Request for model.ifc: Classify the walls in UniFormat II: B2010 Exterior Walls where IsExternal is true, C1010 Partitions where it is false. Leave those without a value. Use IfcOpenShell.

First a look at what the model holds.

```python
import ifcopenshell
import ifcopenshell.util.element

model = ifcopenshell.open("model.ifc")
print(model.schema)
print("classifications:", [c.Name for c in model.by_type("IfcClassification")])
values = [ifcopenshell.util.element.get_pset(e, "Pset_WallCommon", "IsExternal") for e in model.by_type("IfcWall")]
for value in (True, False, None):
    print("IsExternal", value, values.count(value))
```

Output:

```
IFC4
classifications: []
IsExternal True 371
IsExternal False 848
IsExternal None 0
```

```python
import ifcopenshell
import ifcopenshell.api.classification
import ifcopenshell.util.element

model = ifcopenshell.open("model.ifc")

system = ifcopenshell.api.classification.add_classification(model, classification="UniFormat II")

walls = model.by_type("IfcWall")
external = {e: ifcopenshell.util.element.get_pset(e, "Pset_WallCommon", "IsExternal") for e in walls}
for flag, code, name in ((True, "B2010", "Exterior Walls"), (False, "C1010", "Partitions")):
    products = [e for e in walls if external[e] is flag]
    ifcopenshell.api.classification.add_reference(
        model, products=products, classification=system, identification=code, name=name
    )
    print(code, len(products))

model.write("model_updated.ifc")
```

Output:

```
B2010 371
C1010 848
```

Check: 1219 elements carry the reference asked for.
